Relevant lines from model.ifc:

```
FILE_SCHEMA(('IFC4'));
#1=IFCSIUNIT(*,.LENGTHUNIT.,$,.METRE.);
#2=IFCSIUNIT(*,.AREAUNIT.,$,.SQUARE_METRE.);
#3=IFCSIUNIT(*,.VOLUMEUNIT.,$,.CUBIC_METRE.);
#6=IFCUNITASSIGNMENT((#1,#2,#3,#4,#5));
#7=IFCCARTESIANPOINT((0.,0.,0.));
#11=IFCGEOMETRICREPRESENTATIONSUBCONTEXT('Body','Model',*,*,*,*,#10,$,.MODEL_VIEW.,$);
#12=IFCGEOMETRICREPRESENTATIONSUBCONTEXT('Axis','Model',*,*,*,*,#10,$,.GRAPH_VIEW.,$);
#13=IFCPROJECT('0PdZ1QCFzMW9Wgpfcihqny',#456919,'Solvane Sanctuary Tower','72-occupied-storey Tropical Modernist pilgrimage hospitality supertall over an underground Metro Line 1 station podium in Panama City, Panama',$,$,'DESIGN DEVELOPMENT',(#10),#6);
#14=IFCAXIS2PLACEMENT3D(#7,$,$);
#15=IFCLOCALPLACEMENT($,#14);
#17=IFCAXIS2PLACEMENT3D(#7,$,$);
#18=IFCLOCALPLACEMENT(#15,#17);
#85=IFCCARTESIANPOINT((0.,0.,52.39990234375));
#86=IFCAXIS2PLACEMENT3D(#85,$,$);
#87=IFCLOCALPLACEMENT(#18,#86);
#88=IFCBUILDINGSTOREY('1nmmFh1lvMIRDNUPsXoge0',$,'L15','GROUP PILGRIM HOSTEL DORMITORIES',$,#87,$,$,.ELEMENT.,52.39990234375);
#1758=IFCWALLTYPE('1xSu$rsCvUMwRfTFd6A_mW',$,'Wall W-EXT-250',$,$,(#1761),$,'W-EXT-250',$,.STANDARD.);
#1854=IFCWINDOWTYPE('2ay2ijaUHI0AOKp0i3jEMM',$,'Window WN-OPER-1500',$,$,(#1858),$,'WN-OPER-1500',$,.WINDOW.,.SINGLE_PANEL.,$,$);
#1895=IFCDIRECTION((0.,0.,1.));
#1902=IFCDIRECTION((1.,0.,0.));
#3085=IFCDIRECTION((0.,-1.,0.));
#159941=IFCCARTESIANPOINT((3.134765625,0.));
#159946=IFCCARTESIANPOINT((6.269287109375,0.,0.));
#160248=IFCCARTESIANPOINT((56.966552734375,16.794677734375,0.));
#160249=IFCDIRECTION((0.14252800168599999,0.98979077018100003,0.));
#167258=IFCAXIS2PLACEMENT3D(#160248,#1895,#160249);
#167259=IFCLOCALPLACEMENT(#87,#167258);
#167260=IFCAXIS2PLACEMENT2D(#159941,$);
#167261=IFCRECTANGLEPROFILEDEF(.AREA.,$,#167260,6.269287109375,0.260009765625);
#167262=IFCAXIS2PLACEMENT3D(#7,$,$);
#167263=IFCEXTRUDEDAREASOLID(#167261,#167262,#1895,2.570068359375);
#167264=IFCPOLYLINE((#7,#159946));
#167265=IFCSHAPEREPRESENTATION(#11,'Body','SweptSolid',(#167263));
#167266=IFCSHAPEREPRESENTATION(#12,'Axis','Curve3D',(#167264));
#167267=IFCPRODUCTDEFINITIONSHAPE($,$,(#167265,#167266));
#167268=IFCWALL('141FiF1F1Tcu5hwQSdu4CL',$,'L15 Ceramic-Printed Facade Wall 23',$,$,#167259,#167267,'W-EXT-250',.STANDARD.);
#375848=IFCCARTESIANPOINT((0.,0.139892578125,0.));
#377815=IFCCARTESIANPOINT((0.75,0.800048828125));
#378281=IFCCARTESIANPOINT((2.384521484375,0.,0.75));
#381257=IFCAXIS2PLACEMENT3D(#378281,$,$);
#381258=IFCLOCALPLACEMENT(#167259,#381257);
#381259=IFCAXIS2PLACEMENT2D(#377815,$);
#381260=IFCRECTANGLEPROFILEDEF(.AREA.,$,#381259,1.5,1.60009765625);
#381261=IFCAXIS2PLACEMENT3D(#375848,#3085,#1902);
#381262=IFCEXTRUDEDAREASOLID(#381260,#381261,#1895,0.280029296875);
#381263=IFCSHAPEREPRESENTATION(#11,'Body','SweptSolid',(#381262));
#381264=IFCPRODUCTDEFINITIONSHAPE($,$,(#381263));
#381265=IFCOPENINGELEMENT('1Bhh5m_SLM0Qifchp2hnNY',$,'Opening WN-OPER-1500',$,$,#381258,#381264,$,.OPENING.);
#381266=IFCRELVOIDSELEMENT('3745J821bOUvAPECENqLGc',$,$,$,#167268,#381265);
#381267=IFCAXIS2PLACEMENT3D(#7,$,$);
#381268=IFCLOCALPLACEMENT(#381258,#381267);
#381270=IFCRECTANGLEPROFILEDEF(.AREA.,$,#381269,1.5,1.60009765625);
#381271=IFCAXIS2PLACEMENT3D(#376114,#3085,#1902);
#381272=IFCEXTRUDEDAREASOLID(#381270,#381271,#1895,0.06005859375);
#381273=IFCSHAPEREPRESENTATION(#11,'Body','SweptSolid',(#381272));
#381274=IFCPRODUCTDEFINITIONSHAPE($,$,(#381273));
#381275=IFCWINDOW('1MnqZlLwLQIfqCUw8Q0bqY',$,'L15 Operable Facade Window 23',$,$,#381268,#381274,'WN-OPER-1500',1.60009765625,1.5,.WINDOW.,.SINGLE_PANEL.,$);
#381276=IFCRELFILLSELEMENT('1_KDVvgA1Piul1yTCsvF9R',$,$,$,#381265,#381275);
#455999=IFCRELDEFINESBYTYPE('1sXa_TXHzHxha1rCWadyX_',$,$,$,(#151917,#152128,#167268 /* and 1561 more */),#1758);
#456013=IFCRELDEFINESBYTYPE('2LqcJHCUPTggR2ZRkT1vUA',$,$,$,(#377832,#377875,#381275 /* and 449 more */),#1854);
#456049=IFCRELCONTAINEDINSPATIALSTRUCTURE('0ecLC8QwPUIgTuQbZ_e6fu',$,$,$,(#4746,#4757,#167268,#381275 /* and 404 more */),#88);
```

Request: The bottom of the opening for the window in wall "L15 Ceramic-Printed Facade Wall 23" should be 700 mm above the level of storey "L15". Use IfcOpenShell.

```python
import numpy as np
import ifcopenshell
import ifcopenshell.api.geometry
import ifcopenshell.geom
import ifcopenshell.util.element
import ifcopenshell.util.placement
import ifcopenshell.util.shape
import ifcopenshell.util.unit

model = ifcopenshell.open("model.ifc")
unit_scale = ifcopenshell.util.unit.calculate_unit_scale(model)

window = model.by_guid("1MnqZlLwLQIfqCUw8Q0bqY")
opening = window.FillsVoids[0].RelatingOpeningElement
storey = ifcopenshell.util.element.get_container(window, ifc_class="IfcBuildingStorey")
level = ifcopenshell.util.placement.get_local_placement(storey.ObjectPlacement)[2, 3]

# The opening's origin need not be at the sill, so measure its lowest point.
shape = ifcopenshell.geom.create_shape(ifcopenshell.geom.settings(), opening)
bottom = ifcopenshell.util.shape.get_shape_bottom_elevation(shape, shape.geometry) / unit_scale
dz = level + 0.7 / unit_scale - bottom

shift = np.array([0.0, 0.0, dz])
# The window is placed relative to its opening, so it follows when the opening moves.
matrix = ifcopenshell.util.placement.get_local_placement(opening.ObjectPlacement)
matrix[:3, 3] += shift
ifcopenshell.api.geometry.edit_object_placement(
    model, product=opening, matrix=matrix, is_si=False, should_transform_children=True
)

print(f"moved by {dz * unit_scale:+.3f} m")

model.write("model_updated.ifc")
```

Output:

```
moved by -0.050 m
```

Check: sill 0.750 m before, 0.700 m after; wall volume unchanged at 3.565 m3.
